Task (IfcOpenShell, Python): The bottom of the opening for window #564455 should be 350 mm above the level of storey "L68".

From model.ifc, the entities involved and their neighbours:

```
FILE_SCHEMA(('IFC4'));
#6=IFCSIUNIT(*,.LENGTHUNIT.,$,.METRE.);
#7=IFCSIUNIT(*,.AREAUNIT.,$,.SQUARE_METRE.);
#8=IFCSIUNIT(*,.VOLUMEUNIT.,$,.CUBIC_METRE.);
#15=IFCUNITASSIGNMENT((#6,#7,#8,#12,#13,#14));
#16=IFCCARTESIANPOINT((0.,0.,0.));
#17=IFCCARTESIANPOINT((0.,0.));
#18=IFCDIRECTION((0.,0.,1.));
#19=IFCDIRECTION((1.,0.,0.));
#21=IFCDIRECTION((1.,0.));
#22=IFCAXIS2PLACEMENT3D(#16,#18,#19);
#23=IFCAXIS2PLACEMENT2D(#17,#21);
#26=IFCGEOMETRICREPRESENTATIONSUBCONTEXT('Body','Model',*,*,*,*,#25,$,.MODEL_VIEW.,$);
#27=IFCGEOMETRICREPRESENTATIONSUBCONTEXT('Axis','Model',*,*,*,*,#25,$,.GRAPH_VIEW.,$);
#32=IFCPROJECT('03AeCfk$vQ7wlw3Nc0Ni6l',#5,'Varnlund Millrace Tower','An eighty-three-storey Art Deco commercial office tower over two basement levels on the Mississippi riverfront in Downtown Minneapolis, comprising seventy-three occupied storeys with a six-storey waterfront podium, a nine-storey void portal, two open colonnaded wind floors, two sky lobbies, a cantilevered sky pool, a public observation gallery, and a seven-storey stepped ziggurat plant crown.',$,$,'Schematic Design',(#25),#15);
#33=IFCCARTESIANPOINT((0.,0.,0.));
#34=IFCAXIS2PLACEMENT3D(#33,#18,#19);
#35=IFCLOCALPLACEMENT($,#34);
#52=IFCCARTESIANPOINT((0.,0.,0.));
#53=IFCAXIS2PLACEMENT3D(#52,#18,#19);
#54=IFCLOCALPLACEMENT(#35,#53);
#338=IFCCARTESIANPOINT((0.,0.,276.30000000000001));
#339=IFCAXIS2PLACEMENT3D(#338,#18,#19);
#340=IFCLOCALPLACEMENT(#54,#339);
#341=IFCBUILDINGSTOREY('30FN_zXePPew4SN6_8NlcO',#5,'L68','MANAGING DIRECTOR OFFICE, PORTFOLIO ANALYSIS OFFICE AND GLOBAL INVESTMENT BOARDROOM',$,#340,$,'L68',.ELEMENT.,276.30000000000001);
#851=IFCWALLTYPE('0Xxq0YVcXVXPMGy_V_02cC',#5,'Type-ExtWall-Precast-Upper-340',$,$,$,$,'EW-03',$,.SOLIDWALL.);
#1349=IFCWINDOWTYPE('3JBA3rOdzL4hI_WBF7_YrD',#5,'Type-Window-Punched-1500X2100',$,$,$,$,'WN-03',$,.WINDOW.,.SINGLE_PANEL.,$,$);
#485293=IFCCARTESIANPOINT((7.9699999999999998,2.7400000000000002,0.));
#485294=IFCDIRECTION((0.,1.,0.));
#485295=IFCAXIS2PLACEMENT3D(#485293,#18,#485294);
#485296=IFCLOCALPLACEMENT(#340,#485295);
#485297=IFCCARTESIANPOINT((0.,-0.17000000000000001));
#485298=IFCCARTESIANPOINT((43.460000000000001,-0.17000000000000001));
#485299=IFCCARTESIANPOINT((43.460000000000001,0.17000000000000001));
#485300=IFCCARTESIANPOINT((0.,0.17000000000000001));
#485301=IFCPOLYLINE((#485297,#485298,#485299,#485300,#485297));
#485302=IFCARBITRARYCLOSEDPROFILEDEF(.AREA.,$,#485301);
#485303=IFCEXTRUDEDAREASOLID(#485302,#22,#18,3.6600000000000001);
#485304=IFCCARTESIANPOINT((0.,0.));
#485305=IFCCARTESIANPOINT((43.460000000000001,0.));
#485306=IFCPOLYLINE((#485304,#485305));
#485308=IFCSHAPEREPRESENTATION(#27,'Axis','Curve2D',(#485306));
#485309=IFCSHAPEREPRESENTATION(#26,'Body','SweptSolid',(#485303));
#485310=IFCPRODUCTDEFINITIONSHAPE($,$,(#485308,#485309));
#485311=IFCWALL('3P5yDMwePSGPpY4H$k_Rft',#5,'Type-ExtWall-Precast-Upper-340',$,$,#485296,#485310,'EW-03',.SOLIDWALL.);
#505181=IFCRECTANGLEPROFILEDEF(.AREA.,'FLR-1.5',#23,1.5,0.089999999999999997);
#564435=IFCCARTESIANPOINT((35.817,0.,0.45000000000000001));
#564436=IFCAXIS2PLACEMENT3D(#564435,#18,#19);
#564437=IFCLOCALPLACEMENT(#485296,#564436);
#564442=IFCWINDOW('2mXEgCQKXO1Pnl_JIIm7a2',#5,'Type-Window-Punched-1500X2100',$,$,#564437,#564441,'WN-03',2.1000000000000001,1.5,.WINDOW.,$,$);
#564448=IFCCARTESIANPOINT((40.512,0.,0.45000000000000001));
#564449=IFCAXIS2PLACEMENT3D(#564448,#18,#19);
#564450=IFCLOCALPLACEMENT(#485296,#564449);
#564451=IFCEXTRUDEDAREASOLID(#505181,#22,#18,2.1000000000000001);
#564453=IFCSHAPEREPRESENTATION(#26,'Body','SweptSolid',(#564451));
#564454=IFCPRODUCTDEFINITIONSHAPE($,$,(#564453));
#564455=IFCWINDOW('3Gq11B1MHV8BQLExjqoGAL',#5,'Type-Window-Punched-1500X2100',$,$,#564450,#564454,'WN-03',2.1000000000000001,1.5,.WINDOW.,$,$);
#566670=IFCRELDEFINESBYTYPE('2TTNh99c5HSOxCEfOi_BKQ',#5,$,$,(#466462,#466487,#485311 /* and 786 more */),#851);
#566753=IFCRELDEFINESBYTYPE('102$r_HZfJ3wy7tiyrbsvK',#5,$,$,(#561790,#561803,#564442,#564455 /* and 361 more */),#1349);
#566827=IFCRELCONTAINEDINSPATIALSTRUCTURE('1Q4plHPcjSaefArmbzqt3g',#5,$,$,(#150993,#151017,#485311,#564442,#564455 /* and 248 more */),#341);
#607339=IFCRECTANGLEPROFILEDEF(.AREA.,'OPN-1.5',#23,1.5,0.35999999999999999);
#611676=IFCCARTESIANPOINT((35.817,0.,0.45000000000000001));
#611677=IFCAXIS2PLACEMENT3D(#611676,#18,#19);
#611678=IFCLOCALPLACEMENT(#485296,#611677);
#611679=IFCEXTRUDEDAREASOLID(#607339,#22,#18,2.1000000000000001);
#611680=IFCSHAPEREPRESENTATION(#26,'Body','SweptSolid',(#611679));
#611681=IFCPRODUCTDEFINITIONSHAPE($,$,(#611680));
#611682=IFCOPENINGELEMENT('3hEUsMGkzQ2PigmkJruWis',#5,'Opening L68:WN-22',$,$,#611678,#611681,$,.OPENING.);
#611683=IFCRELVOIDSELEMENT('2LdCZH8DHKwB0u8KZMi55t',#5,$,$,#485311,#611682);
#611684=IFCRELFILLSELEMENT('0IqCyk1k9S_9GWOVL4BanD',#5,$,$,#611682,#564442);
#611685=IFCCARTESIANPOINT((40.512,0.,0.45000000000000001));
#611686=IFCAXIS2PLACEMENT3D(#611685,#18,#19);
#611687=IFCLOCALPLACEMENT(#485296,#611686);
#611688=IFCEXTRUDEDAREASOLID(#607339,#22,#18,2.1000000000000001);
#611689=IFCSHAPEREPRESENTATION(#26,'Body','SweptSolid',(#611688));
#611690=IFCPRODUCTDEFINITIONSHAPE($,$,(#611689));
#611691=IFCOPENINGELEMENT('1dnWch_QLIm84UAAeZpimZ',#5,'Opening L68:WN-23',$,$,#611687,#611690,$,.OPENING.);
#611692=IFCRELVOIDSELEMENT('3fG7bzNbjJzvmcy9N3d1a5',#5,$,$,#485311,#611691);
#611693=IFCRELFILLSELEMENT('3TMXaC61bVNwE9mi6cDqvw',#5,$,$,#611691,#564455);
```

```python
import numpy as np
import ifcopenshell
import ifcopenshell.api.geometry
import ifcopenshell.geom
import ifcopenshell.util.element
import ifcopenshell.util.placement
import ifcopenshell.util.shape
import ifcopenshell.util.unit

model = ifcopenshell.open("model.ifc")
unit_scale = ifcopenshell.util.unit.calculate_unit_scale(model)

window = model.by_id(564455)
opening = window.FillsVoids[0].RelatingOpeningElement
storey = ifcopenshell.util.element.get_container(window, ifc_class="IfcBuildingStorey")
level = ifcopenshell.util.placement.get_local_placement(storey.ObjectPlacement)[2, 3]

# The opening's origin need not be at the sill, so measure its lowest point.
shape = ifcopenshell.geom.create_shape(ifcopenshell.geom.settings(), opening)
bottom = ifcopenshell.util.shape.get_shape_bottom_elevation(shape, shape.geometry) / unit_scale
dz = level + 0.35 - bottom

shift = np.array([0.0, 0.0, dz])
# The window is not placed relative to its opening, so move both.
for product in (opening, window):
    matrix = ifcopenshell.util.placement.get_local_placement(product.ObjectPlacement)
    matrix[:3, 3] += shift
    ifcopenshell.api.geometry.edit_object_placement(model, product=product, matrix=matrix, is_si=False)

print(f"moved by {dz * unit_scale:+.3f} m")

model.write("model-out.ifc")
```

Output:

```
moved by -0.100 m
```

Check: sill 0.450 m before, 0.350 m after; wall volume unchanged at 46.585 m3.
